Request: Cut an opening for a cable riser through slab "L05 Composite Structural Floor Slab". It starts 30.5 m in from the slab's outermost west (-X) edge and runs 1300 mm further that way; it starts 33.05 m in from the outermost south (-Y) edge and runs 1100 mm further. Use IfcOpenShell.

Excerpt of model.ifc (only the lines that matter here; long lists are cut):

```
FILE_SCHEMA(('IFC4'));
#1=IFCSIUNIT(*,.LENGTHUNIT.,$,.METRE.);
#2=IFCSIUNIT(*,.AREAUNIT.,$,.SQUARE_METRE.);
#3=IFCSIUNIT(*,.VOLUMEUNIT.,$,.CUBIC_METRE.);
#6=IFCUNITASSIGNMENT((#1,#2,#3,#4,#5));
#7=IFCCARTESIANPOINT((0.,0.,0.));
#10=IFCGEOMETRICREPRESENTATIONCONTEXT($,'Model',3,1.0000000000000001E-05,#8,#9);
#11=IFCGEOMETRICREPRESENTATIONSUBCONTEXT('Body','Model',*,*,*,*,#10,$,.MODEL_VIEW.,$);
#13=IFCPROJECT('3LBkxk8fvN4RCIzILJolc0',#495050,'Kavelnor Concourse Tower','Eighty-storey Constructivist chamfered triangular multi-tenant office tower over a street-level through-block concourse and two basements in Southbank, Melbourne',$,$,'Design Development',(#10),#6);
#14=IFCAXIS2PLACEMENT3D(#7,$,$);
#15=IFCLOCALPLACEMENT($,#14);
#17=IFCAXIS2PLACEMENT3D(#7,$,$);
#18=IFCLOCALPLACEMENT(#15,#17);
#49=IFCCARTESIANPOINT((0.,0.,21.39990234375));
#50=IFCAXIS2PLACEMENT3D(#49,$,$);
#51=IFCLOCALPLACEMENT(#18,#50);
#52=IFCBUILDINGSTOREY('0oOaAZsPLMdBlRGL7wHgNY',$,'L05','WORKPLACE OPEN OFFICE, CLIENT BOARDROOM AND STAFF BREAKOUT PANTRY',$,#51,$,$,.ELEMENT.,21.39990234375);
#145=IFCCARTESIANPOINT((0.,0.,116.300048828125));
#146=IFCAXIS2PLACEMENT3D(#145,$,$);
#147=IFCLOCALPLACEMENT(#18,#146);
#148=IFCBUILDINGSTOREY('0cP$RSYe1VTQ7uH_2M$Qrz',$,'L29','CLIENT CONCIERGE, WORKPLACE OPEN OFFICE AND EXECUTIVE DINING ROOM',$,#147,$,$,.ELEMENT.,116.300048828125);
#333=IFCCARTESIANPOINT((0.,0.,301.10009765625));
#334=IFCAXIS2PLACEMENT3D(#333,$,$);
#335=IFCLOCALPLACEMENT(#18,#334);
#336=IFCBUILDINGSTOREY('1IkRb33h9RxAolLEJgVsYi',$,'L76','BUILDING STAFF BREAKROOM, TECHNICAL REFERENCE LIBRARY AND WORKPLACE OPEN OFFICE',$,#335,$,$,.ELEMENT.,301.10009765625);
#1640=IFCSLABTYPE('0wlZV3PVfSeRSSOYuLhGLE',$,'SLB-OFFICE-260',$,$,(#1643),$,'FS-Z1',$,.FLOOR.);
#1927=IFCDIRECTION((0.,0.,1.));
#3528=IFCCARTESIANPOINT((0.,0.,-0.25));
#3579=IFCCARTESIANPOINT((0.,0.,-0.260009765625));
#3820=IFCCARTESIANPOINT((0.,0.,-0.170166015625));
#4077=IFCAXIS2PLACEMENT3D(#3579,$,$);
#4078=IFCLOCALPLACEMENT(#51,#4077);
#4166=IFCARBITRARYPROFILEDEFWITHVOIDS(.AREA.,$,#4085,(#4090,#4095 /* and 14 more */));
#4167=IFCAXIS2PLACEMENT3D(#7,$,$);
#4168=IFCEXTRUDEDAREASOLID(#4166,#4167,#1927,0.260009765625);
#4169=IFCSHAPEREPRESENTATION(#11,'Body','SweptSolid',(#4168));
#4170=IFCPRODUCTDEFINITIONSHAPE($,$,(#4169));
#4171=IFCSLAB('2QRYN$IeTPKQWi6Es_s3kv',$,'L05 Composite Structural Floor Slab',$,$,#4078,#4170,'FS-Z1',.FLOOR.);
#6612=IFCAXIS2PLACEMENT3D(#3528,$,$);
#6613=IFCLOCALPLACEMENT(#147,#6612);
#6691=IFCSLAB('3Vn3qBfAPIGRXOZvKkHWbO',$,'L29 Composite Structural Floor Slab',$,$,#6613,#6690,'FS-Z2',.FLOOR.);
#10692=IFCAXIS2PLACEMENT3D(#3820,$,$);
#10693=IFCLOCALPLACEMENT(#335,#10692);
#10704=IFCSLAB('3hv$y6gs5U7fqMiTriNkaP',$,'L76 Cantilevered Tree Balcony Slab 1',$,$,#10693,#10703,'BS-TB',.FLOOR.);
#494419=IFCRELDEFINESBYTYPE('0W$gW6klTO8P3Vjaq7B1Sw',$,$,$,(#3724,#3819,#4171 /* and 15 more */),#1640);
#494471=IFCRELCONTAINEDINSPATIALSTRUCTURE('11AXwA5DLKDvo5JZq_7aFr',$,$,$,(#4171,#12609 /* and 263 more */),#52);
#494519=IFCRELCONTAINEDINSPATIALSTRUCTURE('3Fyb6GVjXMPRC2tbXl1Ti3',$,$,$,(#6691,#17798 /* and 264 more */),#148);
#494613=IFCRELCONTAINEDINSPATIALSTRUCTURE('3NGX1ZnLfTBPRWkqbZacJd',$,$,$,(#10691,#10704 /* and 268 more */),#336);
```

```python
import numpy as np
import ifcopenshell
import ifcopenshell.api.feature
import ifcopenshell.api.geometry
import ifcopenshell.api.root
import ifcopenshell.geom
import ifcopenshell.util.placement
import ifcopenshell.util.representation
import ifcopenshell.util.shape
import ifcopenshell.util.unit

model = ifcopenshell.open("model.ifc")
unit_scale = ifcopenshell.util.unit.calculate_unit_scale(model)
settings = ifcopenshell.geom.settings()


def volume(element):
    """Net volume in cubic metres, openings subtracted."""
    shape = ifcopenshell.geom.create_shape(settings, element)
    return ifcopenshell.util.shape.get_volume(shape.geometry)


slab = model.by_guid("2QRYN$IeTPKQWi6Es_s3kv")
before = volume(slab)

# Extent in the slab's own axes, in metres. The edges named are its -X and -Y sides.
slab_shape = ifcopenshell.geom.create_shape(settings, slab)
vertices = ifcopenshell.util.shape.get_vertices(slab_shape.geometry)
x_min, y_min, bottom = vertices.min(axis=0)
top = vertices[:, 2].max()

opening = ifcopenshell.api.root.create_entity(model, ifc_class="IfcOpeningElement", name="Cable riser opening", predefined_type="OPENING")
context = ifcopenshell.util.representation.get_context(model, "Model", "Body", "MODEL_VIEW")
width, depth = 1.3, 1.1
outline = [(0.0, 0.0), (width, 0.0), (width, depth), (0.0, depth), (0.0, 0.0)]
# Overshoot both faces by 50 mm so the cut is clean.
shape = ifcopenshell.api.geometry.add_slab_representation(
    model, context=context, depth=top - bottom + 0.1, polyline=outline
)
ifcopenshell.api.geometry.assign_representation(model, product=opening, representation=shape)

matrix = ifcopenshell.util.placement.get_local_placement(slab.ObjectPlacement)
matrix[:, 3] = matrix @ np.append(np.array([x_min + 30.5, y_min + 33.05, bottom - 0.05]) / unit_scale, 1.0)
ifcopenshell.api.geometry.edit_object_placement(model, product=opening, matrix=matrix, is_si=False)
ifcopenshell.api.feature.add_feature(model, feature=opening, element=slab)

after = volume(slab)

print(f"slab volume {before:.3f} -> {after:.3f} m3")

model.write("model_v2.ifc")
```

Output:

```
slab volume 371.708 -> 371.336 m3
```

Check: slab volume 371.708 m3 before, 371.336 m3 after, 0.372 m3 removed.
